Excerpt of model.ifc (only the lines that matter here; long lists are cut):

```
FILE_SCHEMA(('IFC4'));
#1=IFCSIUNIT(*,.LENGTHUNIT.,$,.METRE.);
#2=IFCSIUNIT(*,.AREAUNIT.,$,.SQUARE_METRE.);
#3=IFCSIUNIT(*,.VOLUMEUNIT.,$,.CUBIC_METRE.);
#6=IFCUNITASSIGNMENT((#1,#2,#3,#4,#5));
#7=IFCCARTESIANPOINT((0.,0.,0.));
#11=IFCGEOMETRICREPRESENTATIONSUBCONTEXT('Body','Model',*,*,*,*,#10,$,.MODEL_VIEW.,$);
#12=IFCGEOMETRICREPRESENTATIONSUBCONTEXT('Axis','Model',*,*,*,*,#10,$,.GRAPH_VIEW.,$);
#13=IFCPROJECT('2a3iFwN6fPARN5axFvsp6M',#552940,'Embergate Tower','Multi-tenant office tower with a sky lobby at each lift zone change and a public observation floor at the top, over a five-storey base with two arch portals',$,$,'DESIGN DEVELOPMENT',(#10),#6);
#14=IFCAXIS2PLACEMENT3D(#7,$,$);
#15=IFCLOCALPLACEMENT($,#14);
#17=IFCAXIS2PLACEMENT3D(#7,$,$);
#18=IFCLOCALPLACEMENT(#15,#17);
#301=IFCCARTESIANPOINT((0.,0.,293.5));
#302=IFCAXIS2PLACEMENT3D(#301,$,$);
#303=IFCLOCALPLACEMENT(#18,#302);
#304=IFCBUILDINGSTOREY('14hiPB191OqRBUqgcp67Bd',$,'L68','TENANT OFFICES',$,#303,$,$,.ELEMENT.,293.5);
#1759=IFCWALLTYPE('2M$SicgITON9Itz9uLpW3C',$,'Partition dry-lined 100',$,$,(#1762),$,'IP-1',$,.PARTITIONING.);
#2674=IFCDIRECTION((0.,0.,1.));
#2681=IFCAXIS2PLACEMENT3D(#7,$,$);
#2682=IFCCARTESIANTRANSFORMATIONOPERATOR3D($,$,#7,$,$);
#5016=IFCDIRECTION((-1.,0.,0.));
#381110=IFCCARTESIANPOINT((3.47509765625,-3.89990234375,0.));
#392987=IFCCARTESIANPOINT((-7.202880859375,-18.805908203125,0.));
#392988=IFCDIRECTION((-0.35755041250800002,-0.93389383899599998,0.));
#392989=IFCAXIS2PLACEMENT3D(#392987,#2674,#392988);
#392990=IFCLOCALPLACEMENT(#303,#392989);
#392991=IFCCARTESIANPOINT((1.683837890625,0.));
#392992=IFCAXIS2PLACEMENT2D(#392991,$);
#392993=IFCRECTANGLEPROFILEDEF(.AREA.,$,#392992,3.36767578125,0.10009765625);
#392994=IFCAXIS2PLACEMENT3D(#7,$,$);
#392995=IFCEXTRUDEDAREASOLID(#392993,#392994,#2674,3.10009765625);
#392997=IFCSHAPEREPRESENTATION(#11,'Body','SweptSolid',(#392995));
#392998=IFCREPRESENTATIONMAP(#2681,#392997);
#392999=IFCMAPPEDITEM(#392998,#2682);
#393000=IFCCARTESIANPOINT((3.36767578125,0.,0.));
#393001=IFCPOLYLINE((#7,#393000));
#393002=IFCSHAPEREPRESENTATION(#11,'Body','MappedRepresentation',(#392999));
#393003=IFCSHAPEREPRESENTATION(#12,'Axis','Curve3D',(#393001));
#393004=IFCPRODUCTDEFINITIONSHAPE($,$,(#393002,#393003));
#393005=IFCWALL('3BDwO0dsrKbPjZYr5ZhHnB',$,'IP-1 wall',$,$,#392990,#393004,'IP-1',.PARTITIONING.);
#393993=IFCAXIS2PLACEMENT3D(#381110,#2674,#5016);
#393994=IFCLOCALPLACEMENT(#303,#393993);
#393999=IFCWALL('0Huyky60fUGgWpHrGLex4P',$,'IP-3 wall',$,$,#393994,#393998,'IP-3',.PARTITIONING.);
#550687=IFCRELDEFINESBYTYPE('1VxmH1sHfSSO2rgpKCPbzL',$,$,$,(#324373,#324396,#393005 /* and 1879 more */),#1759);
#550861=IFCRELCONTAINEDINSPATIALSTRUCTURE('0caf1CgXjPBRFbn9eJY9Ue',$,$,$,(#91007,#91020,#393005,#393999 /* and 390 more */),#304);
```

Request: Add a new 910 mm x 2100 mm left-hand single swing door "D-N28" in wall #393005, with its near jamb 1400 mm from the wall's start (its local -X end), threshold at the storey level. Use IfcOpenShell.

```python
import numpy as np
import ifcopenshell
import ifcopenshell.api.feature
import ifcopenshell.api.geometry
import ifcopenshell.api.root
import ifcopenshell.api.spatial
import ifcopenshell.geom
import ifcopenshell.util.element
import ifcopenshell.util.placement
import ifcopenshell.util.representation
import ifcopenshell.util.shape
import ifcopenshell.util.unit

model = ifcopenshell.open("model.ifc")
unit_scale = ifcopenshell.util.unit.calculate_unit_scale(model)
settings = ifcopenshell.geom.settings()


def volume(element):
    """Net volume in cubic metres, openings subtracted."""
    shape = ifcopenshell.geom.create_shape(settings, element)
    return ifcopenshell.util.shape.get_volume(shape.geometry)


wall = model.by_id(393005)
storey = ifcopenshell.util.element.get_container(wall, ifc_class="IfcBuildingStorey")
context = ifcopenshell.util.representation.get_context(model, "Model", "Body", "MODEL_VIEW")
before = volume(wall)

width, height, from_end, sill = 0.91, 2.1, 1.4, 0.0  # metres

# The wall runs along its own X axis, and the end named is its -X end.
wall_shape = ifcopenshell.geom.create_shape(settings, wall)
x, y, z = ifcopenshell.util.shape.get_vertices(wall_shape.geometry).T
start = x.min() + from_end
face, thickness = float(y.min()), float(y.max() - y.min())
wall_matrix = ifcopenshell.util.placement.get_local_placement(wall.ObjectPlacement)
level = ifcopenshell.util.placement.get_local_placement(storey.ObjectPlacement)[2, 3]


def in_wall(x, y):
    """Placement at x, y metres in the wall's axes, at sill height."""
    matrix = wall_matrix.copy()
    matrix[:, 3] = wall_matrix @ np.array([x / unit_scale, y / unit_scale, 0.0, 1.0])
    matrix[2, 3] = level + sill / unit_scale
    return matrix


# Opening: a box that overshoots both wall faces by 50 mm.
opening = ifcopenshell.api.root.create_entity(model, ifc_class="IfcOpeningElement", predefined_type="OPENING")
box = ifcopenshell.api.geometry.add_wall_representation(
    model, context=context, length=width, height=height, thickness=thickness + 0.1
)
ifcopenshell.api.geometry.assign_representation(model, product=opening, representation=box)
ifcopenshell.api.geometry.edit_object_placement(model, product=opening, matrix=in_wall(start, face - 0.05), is_si=False)
ifcopenshell.api.feature.add_feature(model, feature=opening, element=wall)

door = ifcopenshell.api.root.create_entity(model, ifc_class="IfcDoor", name="D-N28", predefined_type="DOOR")
door.OverallWidth, door.OverallHeight = width / unit_scale, height / unit_scale
door.OperationType = "SINGLE_SWING_LEFT"
body = ifcopenshell.api.geometry.add_door_representation(
    model,
    context=context,
    overall_width=door.OverallWidth,
    overall_height=door.OverallHeight,
    operation_type="SINGLE_SWING_LEFT",
    lining_properties={"LiningDepth": thickness / unit_scale, "ThresholdDepth": thickness / unit_scale},
)
ifcopenshell.api.geometry.assign_representation(model, product=door, representation=body)
ifcopenshell.api.spatial.assign_container(model, products=[door], relating_structure=storey)
ifcopenshell.api.feature.add_filling(model, opening=opening, element=door)

# The lining spans the wall, so the door starts at the wall face.
ifcopenshell.api.geometry.edit_object_placement(model, product=door, matrix=in_wall(start, face), is_si=False)

after = volume(wall)

print(f"wall volume {before:.3f} -> {after:.3f} m3")

model.write("model-out.ifc")
```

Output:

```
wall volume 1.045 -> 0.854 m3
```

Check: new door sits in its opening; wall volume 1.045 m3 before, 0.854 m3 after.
